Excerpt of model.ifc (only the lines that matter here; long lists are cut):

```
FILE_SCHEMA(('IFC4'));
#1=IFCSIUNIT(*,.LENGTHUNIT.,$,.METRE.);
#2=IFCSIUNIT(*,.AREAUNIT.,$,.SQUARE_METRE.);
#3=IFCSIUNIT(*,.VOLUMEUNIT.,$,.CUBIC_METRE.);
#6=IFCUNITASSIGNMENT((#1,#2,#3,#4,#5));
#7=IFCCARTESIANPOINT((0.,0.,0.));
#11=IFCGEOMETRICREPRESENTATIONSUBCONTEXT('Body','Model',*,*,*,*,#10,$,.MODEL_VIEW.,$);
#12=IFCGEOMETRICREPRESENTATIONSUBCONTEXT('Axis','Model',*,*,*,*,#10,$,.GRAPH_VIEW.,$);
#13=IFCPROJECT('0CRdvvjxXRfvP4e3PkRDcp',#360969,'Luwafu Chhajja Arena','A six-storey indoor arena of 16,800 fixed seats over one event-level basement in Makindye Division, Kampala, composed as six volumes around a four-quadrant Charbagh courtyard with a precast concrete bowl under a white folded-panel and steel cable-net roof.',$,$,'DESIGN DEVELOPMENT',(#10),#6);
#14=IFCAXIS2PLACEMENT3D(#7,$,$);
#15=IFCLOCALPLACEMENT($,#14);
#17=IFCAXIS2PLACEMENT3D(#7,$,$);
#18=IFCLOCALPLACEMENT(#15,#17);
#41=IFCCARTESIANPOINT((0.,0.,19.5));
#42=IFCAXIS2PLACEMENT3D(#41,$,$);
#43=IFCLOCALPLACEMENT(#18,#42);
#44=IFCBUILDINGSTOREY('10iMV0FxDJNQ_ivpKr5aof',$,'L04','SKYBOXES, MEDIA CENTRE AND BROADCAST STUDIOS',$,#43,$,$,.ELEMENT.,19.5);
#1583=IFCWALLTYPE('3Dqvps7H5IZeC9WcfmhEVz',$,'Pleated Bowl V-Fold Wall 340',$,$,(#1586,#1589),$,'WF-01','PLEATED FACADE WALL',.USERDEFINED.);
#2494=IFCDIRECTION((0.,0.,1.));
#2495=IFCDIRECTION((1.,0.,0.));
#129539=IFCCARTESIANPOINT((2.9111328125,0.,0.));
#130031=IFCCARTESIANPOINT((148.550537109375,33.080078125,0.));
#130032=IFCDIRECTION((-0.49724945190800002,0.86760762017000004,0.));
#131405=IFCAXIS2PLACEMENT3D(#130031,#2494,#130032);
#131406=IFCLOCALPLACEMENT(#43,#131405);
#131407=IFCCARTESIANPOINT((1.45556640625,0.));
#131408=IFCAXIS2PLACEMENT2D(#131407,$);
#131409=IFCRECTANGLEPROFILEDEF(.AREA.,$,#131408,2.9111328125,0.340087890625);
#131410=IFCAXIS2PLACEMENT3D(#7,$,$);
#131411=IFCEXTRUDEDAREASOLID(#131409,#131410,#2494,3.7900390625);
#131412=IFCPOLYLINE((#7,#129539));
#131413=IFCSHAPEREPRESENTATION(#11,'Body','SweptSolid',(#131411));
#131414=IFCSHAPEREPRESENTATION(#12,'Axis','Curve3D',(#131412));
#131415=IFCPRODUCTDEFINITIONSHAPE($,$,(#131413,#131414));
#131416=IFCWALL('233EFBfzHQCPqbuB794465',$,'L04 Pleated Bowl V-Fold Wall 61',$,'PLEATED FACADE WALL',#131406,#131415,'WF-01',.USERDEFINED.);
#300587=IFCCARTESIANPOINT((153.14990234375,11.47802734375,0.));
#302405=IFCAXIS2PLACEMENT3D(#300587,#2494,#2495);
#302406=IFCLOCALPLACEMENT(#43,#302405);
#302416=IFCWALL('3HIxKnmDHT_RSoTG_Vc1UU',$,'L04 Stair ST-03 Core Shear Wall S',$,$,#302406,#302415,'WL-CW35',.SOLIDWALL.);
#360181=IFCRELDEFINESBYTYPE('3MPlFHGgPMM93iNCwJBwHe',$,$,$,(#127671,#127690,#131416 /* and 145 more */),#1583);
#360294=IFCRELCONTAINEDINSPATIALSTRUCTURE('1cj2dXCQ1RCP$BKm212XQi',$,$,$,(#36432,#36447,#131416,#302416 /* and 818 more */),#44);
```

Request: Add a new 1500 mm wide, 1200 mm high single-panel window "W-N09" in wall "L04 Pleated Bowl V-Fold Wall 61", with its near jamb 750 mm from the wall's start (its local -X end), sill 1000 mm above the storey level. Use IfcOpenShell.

```python
import numpy as np
import ifcopenshell
import ifcopenshell.api.feature
import ifcopenshell.api.geometry
import ifcopenshell.api.root
import ifcopenshell.api.spatial
import ifcopenshell.geom
import ifcopenshell.util.element
import ifcopenshell.util.placement
import ifcopenshell.util.representation
import ifcopenshell.util.shape
import ifcopenshell.util.unit

model = ifcopenshell.open("model.ifc")
unit_scale = ifcopenshell.util.unit.calculate_unit_scale(model)
settings = ifcopenshell.geom.settings()


def volume(element):
    """Net volume in cubic metres, openings subtracted."""
    shape = ifcopenshell.geom.create_shape(settings, element)
    return ifcopenshell.util.shape.get_volume(shape.geometry)


wall = model.by_guid("233EFBfzHQCPqbuB794465")
storey = ifcopenshell.util.element.get_container(wall, ifc_class="IfcBuildingStorey")
context = ifcopenshell.util.representation.get_context(model, "Model", "Body", "MODEL_VIEW")
before = volume(wall)

width, height, from_end, sill = 1.5, 1.2, 0.75, 1  # metres

# The wall runs along its own X axis, and the end named is its -X end.
wall_shape = ifcopenshell.geom.create_shape(settings, wall)
x, y, z = ifcopenshell.util.shape.get_vertices(wall_shape.geometry).T
start = x.min() + from_end
face, thickness = float(y.min()), float(y.max() - y.min())
wall_matrix = ifcopenshell.util.placement.get_local_placement(wall.ObjectPlacement)
level = ifcopenshell.util.placement.get_local_placement(storey.ObjectPlacement)[2, 3]


def in_wall(x, y):
    """Placement at x, y metres in the wall's axes, at sill height."""
    matrix = wall_matrix.copy()
    matrix[:, 3] = wall_matrix @ np.array([x / unit_scale, y / unit_scale, 0.0, 1.0])
    matrix[2, 3] = level + sill / unit_scale
    return matrix


# Opening: a box that overshoots both wall faces by 50 mm.
opening = ifcopenshell.api.root.create_entity(model, ifc_class="IfcOpeningElement", predefined_type="OPENING")
box = ifcopenshell.api.geometry.add_wall_representation(
    model, context=context, length=width, height=height, thickness=thickness + 0.1
)
ifcopenshell.api.geometry.assign_representation(model, product=opening, representation=box)
ifcopenshell.api.geometry.edit_object_placement(model, product=opening, matrix=in_wall(start, face - 0.05), is_si=False)
ifcopenshell.api.feature.add_feature(model, feature=opening, element=wall)

window = ifcopenshell.api.root.create_entity(model, ifc_class="IfcWindow", name="W-N09", predefined_type="WINDOW")
window.OverallWidth, window.OverallHeight = width / unit_scale, height / unit_scale
window.PartitioningType = "SINGLE_PANEL"
body = ifcopenshell.api.geometry.add_window_representation(
    model,
    context=context,
    overall_width=window.OverallWidth,
    overall_height=window.OverallHeight,
    partition_type="SINGLE_PANEL",
)
ifcopenshell.api.geometry.assign_representation(model, product=window, representation=body)
ifcopenshell.api.spatial.assign_container(model, products=[window], relating_structure=storey)
ifcopenshell.api.feature.add_filling(model, opening=opening, element=window)

# Centre the window in the wall's thickness.
ifcopenshell.api.geometry.edit_object_placement(model, product=window, matrix=in_wall(start, face), is_si=False)
window_shape = ifcopenshell.geom.create_shape(settings, window)
depth = ifcopenshell.util.shape.get_vertices(window_shape.geometry)[:, 1]
offset = face + thickness / 2 - (depth.min() + depth.max()) / 2
ifcopenshell.api.geometry.edit_object_placement(model, product=window, matrix=in_wall(start, offset), is_si=False)

after = volume(wall)

print(f"wall volume {before:.3f} -> {after:.3f} m3")

model.write("model_v2.ifc")
```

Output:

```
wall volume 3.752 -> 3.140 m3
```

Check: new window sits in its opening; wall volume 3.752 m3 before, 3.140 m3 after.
